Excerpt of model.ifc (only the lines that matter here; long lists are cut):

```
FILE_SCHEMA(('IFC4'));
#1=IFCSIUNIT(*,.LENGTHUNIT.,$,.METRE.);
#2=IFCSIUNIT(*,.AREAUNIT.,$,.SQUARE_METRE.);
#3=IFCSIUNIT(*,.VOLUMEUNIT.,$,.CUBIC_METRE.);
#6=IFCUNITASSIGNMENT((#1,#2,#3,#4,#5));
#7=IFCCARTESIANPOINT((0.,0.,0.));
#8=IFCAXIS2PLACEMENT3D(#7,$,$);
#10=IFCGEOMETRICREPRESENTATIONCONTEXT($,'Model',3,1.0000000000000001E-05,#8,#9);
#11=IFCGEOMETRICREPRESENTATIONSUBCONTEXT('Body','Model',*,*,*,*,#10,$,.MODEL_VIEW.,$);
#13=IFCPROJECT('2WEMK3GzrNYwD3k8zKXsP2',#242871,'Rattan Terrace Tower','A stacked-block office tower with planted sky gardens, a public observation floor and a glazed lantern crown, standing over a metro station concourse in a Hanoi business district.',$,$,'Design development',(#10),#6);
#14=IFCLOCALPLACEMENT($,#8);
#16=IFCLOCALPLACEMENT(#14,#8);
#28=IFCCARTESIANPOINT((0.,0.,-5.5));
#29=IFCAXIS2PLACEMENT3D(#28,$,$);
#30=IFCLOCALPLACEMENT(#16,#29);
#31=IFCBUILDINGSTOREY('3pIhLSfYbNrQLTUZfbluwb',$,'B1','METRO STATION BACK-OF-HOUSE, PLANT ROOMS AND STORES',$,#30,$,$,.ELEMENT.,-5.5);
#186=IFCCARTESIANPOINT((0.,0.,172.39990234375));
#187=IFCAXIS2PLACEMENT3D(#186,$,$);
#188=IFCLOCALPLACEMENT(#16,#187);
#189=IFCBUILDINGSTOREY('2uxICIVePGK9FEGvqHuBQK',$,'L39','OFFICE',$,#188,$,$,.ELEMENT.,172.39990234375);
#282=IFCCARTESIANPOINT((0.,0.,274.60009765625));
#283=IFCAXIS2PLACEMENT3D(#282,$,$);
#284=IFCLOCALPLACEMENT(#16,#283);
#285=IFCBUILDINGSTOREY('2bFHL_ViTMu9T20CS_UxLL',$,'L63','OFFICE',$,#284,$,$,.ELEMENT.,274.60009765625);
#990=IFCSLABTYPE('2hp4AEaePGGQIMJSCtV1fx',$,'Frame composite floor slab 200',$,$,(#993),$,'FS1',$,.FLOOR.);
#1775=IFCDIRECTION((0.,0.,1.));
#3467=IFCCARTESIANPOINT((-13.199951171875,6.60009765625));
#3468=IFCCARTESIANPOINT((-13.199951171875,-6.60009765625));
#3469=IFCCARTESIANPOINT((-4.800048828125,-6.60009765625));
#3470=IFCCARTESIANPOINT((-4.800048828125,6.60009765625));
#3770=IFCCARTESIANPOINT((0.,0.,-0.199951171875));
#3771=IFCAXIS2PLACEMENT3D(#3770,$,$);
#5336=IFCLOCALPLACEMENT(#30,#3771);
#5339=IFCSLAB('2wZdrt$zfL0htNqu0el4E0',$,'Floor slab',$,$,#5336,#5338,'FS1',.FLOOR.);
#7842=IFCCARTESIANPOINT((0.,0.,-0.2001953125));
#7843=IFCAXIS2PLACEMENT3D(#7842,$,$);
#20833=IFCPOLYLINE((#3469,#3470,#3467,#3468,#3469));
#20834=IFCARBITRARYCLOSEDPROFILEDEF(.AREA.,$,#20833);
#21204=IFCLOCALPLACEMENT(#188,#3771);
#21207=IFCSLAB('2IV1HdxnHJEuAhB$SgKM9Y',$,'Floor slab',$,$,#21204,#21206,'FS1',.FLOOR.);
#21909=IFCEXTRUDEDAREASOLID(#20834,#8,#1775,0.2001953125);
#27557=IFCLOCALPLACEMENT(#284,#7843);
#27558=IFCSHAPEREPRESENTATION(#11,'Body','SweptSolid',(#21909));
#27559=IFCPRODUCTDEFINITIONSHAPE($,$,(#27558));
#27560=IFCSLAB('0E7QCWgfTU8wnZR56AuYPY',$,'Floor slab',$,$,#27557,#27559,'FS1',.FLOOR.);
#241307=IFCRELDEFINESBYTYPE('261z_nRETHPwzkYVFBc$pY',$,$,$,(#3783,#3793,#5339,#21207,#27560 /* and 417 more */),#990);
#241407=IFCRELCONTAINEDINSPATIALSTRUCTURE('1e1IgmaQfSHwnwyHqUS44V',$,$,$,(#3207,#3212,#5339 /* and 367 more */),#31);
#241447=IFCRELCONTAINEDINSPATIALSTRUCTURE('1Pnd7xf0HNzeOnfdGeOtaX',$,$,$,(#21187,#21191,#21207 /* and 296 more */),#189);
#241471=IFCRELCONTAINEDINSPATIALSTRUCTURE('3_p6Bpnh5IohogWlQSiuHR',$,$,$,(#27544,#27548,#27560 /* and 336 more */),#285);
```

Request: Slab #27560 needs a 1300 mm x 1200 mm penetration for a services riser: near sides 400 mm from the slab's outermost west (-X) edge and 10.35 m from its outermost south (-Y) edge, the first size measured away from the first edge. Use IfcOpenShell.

```python
import numpy as np
import ifcopenshell
import ifcopenshell.api.feature
import ifcopenshell.api.geometry
import ifcopenshell.api.root
import ifcopenshell.geom
import ifcopenshell.util.placement
import ifcopenshell.util.representation
import ifcopenshell.util.shape
import ifcopenshell.util.unit

model = ifcopenshell.open("model.ifc")
unit_scale = ifcopenshell.util.unit.calculate_unit_scale(model)
settings = ifcopenshell.geom.settings()


def volume(element):
    """Net volume in cubic metres, openings subtracted."""
    shape = ifcopenshell.geom.create_shape(settings, element)
    return ifcopenshell.util.shape.get_volume(shape.geometry)


slab = model.by_id(27560)
before = volume(slab)

# Extent in the slab's own axes, in metres. The edges named are its -X and -Y sides.
slab_shape = ifcopenshell.geom.create_shape(settings, slab)
vertices = ifcopenshell.util.shape.get_vertices(slab_shape.geometry)
x_min, y_min, bottom = vertices.min(axis=0)
top = vertices[:, 2].max()

opening = ifcopenshell.api.root.create_entity(model, ifc_class="IfcOpeningElement", name="Services riser opening", predefined_type="OPENING")
context = ifcopenshell.util.representation.get_context(model, "Model", "Body", "MODEL_VIEW")
width, depth = 1.3, 1.2
outline = [(0.0, 0.0), (width, 0.0), (width, depth), (0.0, depth), (0.0, 0.0)]
# Overshoot both faces by 50 mm so the cut is clean.
shape = ifcopenshell.api.geometry.add_slab_representation(
    model, context=context, depth=top - bottom + 0.1, polyline=outline
)
ifcopenshell.api.geometry.assign_representation(model, product=opening, representation=shape)

matrix = ifcopenshell.util.placement.get_local_placement(slab.ObjectPlacement)
matrix[:, 3] = matrix @ np.append(np.array([x_min + 0.4, y_min + 10.35, bottom - 0.05]) / unit_scale, 1.0)
ifcopenshell.api.geometry.edit_object_placement(model, product=opening, matrix=matrix, is_si=False)
ifcopenshell.api.feature.add_feature(model, feature=opening, element=slab)

after = volume(slab)

print(f"slab volume {before:.3f} -> {after:.3f} m3")

model.write("model_updated.ifc")
```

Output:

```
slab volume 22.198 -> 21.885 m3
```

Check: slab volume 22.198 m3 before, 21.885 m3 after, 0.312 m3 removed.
